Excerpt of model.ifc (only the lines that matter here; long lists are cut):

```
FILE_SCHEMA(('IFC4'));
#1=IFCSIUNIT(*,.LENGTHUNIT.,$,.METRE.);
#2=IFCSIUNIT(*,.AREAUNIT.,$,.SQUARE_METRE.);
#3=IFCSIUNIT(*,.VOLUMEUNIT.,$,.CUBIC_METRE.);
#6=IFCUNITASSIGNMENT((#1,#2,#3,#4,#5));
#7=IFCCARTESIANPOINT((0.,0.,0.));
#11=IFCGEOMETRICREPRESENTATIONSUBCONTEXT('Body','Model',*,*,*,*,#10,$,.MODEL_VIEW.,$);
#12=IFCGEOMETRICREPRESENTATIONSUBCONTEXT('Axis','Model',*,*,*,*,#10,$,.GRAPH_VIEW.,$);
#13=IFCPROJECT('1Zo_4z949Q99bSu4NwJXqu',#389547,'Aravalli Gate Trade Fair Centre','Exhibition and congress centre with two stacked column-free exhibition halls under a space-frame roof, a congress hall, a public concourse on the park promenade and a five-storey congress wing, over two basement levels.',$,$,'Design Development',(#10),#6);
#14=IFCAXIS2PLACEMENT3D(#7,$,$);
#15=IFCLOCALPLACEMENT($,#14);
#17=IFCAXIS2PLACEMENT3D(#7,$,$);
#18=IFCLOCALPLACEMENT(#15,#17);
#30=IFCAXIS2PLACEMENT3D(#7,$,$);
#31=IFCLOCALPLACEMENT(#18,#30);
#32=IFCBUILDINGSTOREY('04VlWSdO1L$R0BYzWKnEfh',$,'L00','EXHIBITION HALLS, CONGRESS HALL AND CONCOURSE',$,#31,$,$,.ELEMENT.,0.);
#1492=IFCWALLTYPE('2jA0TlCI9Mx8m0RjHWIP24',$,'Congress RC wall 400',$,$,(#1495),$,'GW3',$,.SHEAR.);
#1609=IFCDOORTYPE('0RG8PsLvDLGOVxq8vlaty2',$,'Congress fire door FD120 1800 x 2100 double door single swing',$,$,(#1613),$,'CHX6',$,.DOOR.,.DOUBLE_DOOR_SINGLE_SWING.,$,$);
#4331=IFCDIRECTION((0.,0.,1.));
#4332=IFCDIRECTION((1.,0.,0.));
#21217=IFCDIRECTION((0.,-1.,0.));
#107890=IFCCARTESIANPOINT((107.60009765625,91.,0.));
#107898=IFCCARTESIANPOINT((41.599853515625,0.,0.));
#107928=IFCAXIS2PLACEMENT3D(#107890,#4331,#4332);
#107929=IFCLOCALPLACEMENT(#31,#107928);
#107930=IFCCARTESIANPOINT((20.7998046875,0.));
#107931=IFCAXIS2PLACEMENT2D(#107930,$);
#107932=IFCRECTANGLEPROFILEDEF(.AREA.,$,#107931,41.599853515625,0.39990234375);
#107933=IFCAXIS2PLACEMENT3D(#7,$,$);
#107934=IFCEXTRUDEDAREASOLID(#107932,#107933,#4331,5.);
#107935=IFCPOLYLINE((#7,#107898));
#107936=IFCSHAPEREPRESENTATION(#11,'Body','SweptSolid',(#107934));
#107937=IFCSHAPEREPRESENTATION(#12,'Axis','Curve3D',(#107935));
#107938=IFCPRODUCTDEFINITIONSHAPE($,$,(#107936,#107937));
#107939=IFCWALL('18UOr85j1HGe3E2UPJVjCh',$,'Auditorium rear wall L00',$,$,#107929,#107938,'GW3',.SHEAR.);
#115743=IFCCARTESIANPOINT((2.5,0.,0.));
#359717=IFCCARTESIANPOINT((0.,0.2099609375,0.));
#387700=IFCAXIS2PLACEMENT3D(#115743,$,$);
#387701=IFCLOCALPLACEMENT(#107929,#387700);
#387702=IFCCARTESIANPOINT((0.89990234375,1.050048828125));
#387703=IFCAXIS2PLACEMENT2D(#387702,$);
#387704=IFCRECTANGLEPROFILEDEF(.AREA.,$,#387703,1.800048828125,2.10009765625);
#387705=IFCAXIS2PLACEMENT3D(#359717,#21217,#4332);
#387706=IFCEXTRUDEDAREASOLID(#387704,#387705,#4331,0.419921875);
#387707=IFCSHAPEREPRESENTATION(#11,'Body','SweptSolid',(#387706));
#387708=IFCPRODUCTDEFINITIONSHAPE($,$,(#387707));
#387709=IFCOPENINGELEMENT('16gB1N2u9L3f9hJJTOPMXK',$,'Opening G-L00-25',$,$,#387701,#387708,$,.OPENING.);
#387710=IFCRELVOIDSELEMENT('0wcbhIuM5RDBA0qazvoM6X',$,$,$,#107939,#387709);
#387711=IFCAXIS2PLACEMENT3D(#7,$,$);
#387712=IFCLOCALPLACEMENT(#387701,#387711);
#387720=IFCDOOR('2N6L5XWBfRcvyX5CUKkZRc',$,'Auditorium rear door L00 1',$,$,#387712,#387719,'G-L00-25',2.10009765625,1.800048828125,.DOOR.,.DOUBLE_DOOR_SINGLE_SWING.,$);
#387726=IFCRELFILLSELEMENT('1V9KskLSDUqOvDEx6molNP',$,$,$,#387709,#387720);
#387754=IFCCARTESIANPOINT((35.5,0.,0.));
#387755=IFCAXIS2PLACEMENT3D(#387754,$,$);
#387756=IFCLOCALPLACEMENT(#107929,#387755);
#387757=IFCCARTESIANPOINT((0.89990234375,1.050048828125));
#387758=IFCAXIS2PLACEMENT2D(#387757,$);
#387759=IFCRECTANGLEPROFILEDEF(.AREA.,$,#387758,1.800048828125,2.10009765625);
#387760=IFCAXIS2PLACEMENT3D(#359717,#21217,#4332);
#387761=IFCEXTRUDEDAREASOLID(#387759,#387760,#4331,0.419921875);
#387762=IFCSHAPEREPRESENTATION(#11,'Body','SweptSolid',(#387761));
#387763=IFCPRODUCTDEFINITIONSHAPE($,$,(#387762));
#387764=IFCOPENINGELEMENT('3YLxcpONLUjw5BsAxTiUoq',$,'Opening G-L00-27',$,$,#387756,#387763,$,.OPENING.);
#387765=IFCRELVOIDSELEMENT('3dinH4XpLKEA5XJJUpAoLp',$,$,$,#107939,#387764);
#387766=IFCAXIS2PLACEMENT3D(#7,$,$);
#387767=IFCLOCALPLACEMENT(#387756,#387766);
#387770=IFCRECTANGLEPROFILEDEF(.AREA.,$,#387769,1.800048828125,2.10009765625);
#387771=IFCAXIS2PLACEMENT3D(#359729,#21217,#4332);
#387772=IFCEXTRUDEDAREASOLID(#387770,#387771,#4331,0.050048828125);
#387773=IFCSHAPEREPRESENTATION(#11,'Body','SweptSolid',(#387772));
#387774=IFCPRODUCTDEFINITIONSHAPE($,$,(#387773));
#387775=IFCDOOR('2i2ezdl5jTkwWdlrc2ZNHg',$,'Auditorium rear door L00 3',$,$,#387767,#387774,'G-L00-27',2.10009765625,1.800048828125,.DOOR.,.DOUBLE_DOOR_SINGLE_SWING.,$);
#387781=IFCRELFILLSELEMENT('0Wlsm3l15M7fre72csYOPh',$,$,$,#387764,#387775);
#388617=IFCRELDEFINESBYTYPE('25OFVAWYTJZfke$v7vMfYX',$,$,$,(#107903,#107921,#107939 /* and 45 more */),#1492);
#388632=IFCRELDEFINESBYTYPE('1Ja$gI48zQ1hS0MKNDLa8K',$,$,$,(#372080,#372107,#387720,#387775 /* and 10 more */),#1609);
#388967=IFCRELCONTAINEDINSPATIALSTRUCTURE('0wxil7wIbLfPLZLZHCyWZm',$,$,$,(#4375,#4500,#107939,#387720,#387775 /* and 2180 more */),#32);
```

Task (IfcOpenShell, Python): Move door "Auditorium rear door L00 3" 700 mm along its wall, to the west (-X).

```python
import ifcopenshell
import ifcopenshell.api.geometry
import ifcopenshell.util.placement

model = ifcopenshell.open("model.ifc")

door = model.by_id(387775)
opening = door.FillsVoids[0].RelatingOpeningElement
wall = opening.VoidsElements[0].RelatingBuildingElement

wall_matrix = ifcopenshell.util.placement.get_local_placement(wall.ObjectPlacement)
shift = wall_matrix[:3, 0] * -0.7
before = ifcopenshell.util.placement.get_local_placement(door.ObjectPlacement)[:3, 3].copy()

# The door is placed relative to its opening, so it follows when the opening moves.
matrix = ifcopenshell.util.placement.get_local_placement(opening.ObjectPlacement)
matrix[:3, 3] += shift
ifcopenshell.api.geometry.edit_object_placement(
    model, product=opening, matrix=matrix, is_si=False, should_transform_children=True
)

after = ifcopenshell.util.placement.get_local_placement(door.ObjectPlacement)[:3, 3]
print("door moved by", (after - before).round(3) + 0.0)

model.write("model_updated.ifc")
```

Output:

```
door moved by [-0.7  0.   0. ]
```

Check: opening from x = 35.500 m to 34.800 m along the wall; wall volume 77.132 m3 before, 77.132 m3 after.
